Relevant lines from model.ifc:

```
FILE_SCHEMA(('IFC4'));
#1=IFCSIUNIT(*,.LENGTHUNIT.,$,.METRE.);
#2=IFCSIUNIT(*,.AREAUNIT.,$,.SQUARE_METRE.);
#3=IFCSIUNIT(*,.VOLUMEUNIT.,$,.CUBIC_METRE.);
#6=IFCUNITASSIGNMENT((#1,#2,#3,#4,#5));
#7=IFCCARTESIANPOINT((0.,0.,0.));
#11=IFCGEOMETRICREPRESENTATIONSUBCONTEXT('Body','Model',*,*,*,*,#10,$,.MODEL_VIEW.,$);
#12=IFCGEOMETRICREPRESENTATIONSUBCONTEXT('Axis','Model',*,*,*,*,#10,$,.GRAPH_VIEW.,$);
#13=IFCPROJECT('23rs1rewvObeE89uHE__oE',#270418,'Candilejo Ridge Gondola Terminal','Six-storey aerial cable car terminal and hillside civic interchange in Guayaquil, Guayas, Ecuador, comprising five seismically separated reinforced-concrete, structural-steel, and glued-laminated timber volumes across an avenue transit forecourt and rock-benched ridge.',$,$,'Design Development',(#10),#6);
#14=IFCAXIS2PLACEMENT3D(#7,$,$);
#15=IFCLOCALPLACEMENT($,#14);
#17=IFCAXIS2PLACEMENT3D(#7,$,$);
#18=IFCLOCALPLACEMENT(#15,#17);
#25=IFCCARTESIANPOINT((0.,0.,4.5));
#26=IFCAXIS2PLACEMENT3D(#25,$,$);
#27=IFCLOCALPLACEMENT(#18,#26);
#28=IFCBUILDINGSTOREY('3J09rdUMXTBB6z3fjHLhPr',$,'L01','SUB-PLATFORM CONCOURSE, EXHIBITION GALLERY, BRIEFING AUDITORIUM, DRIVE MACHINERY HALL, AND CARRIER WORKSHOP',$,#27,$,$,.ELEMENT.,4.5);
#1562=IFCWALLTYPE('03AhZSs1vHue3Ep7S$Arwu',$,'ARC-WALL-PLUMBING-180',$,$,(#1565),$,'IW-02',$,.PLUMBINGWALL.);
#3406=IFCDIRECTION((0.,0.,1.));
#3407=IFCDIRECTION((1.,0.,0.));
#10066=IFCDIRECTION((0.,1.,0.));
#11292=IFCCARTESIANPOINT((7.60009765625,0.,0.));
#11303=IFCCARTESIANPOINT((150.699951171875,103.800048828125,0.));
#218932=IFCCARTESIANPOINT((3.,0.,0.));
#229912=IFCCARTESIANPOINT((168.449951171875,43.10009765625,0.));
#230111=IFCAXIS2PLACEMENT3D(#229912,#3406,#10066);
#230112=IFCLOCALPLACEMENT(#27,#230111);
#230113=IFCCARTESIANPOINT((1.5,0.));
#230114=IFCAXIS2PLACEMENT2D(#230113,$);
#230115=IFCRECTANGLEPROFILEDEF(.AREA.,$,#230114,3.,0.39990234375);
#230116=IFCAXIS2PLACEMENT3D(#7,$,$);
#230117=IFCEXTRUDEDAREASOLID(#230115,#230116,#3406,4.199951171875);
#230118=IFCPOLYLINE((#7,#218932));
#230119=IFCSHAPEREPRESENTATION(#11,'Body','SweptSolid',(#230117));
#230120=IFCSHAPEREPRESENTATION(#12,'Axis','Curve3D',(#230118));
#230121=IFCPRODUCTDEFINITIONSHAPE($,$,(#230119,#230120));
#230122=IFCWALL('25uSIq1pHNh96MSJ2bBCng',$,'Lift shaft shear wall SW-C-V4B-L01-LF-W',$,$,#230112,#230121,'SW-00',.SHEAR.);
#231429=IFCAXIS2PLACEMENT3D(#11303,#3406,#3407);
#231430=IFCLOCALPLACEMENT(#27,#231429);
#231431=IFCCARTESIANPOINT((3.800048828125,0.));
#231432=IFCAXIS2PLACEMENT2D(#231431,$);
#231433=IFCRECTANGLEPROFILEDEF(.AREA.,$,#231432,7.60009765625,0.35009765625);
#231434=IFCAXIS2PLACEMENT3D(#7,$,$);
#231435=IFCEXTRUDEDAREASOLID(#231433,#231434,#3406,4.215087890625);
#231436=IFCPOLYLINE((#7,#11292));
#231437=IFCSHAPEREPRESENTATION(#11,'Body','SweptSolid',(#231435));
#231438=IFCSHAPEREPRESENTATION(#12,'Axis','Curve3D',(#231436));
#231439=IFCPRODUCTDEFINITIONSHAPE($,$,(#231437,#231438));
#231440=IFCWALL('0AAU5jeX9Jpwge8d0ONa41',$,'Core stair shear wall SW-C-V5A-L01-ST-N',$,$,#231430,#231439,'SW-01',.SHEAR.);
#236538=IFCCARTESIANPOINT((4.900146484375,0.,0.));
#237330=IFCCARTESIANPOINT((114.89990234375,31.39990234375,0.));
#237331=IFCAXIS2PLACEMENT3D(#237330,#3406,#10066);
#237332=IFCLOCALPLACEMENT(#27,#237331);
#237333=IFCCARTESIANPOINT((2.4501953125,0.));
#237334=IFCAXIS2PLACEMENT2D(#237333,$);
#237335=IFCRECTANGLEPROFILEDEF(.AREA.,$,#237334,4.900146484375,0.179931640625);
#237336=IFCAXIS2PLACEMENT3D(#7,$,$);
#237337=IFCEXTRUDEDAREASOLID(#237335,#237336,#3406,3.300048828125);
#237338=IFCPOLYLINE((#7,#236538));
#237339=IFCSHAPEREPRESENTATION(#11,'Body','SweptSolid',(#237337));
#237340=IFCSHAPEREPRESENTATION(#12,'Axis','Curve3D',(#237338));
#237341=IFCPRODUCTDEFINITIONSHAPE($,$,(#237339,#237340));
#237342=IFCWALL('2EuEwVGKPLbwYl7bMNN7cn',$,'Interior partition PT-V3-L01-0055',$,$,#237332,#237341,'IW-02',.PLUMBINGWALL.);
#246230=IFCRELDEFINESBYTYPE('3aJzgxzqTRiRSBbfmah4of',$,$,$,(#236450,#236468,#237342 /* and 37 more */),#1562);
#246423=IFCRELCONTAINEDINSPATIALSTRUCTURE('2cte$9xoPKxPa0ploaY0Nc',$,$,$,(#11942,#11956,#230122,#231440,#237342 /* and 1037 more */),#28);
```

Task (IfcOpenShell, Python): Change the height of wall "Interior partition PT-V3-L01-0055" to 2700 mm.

```python
import ifcopenshell
import ifcopenshell.geom
import ifcopenshell.util.representation
import ifcopenshell.util.shape

model = ifcopenshell.open("model.ifc")
settings = ifcopenshell.geom.settings()


def volume(element):
    """Net volume in cubic metres, openings subtracted."""
    shape = ifcopenshell.geom.create_shape(settings, element)
    return ifcopenshell.util.shape.get_volume(shape.geometry)


wall = model.by_guid("2EuEwVGKPLbwYl7bMNN7cn")
before = volume(wall)

body = ifcopenshell.util.representation.get_representation(wall, "Model", "Body")
solid = body.Items[0]
old_height = solid.Depth
solid.Depth = 2.7
after = volume(wall)

print(f"height {old_height:g} -> {solid.Depth:g}, volume {before:.3f} -> {after:.3f} m3")

model.write("model_v2.ifc")
```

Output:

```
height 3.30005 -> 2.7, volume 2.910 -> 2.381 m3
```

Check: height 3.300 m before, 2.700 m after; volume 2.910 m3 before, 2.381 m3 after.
